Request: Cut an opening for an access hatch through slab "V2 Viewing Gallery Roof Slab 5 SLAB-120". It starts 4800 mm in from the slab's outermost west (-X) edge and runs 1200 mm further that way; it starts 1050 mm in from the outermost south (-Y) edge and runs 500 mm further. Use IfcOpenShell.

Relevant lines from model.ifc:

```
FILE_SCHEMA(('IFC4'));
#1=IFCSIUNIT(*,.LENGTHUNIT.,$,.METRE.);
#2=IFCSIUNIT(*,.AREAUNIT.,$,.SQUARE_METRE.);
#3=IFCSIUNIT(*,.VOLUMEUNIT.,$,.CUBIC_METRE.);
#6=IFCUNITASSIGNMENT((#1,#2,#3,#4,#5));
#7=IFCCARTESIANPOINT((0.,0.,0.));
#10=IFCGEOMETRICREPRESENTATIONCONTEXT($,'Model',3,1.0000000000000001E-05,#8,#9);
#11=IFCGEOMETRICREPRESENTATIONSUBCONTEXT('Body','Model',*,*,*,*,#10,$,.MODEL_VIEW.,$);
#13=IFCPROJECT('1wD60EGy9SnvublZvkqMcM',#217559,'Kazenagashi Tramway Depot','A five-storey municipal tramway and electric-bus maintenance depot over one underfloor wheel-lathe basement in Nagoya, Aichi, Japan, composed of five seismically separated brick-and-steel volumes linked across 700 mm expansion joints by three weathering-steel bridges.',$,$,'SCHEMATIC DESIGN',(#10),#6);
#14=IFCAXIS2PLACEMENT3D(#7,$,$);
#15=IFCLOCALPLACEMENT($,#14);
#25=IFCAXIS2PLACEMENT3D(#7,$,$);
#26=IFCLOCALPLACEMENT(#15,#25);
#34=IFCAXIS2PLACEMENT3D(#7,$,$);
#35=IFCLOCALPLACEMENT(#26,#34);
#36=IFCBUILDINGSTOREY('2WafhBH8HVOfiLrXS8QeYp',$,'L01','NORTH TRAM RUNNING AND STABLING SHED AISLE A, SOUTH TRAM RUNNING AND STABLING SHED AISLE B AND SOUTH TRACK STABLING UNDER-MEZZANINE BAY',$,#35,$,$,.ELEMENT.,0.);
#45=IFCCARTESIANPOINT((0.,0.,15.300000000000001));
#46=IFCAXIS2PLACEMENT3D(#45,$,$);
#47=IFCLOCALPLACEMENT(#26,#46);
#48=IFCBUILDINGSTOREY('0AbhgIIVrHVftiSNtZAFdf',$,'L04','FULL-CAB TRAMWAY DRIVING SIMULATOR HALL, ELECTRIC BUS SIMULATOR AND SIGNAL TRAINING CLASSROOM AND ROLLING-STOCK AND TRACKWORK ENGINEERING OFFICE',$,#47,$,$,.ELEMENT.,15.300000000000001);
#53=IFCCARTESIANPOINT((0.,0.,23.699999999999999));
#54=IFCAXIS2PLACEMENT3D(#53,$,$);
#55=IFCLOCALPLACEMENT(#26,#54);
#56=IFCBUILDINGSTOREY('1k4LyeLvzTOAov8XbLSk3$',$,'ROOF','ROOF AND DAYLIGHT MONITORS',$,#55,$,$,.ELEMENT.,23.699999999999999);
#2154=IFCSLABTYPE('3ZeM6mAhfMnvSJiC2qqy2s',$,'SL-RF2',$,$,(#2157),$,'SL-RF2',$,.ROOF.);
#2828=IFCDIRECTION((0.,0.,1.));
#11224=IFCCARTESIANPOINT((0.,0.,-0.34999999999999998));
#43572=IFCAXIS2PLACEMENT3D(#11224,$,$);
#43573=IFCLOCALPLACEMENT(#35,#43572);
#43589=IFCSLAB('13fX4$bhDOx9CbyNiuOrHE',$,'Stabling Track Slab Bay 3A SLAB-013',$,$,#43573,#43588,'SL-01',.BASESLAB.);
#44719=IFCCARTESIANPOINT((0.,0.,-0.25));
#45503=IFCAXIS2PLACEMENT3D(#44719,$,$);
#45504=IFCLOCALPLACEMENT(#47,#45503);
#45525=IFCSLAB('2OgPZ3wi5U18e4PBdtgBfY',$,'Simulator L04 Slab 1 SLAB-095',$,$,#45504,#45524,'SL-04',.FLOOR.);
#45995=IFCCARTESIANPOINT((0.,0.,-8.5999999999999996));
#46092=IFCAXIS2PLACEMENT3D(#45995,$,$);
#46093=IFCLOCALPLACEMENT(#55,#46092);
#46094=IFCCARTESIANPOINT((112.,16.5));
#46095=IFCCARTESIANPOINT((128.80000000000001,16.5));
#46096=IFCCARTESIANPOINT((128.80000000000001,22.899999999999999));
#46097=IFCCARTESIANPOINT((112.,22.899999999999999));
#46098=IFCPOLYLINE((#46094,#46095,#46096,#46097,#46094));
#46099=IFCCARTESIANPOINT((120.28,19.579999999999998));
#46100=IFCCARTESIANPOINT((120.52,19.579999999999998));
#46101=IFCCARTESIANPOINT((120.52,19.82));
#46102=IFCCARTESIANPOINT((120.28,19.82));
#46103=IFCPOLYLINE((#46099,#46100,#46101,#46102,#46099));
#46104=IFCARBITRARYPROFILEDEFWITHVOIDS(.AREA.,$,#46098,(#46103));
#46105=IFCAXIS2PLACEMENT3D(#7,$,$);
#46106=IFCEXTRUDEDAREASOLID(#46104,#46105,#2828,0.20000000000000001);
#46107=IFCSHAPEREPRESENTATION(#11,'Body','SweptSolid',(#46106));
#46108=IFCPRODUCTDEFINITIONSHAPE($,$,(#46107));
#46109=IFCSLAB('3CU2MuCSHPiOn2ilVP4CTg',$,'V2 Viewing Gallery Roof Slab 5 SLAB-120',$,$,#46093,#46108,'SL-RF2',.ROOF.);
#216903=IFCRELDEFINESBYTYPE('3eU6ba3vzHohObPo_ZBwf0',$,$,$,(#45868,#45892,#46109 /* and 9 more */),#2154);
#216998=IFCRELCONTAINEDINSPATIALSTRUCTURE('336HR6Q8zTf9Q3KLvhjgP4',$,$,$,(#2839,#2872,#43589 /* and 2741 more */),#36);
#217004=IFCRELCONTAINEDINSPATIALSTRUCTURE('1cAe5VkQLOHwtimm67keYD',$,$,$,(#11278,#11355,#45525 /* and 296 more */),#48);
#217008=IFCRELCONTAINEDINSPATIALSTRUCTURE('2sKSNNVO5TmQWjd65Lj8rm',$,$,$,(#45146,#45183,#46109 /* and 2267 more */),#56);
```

```python
import numpy as np
import ifcopenshell
import ifcopenshell.api.feature
import ifcopenshell.api.geometry
import ifcopenshell.api.root
import ifcopenshell.geom
import ifcopenshell.util.placement
import ifcopenshell.util.representation
import ifcopenshell.util.shape
import ifcopenshell.util.unit

model = ifcopenshell.open("model.ifc")
unit_scale = ifcopenshell.util.unit.calculate_unit_scale(model)
settings = ifcopenshell.geom.settings()


def volume(element):
    """Net volume in cubic metres, openings subtracted."""
    shape = ifcopenshell.geom.create_shape(settings, element)
    return ifcopenshell.util.shape.get_volume(shape.geometry)


slab = model.by_id(46109)
before = volume(slab)

# Extent in the slab's own axes, in metres. The edges named are its -X and -Y sides.
slab_shape = ifcopenshell.geom.create_shape(settings, slab)
vertices = ifcopenshell.util.shape.get_vertices(slab_shape.geometry)
x_min, y_min, bottom = vertices.min(axis=0)
top = vertices[:, 2].max()

opening = ifcopenshell.api.root.create_entity(model, ifc_class="IfcOpeningElement", name="Access hatch opening", predefined_type="OPENING")
context = ifcopenshell.util.representation.get_context(model, "Model", "Body", "MODEL_VIEW")
width, depth = 1.2, 0.5
outline = [(0.0, 0.0), (width, 0.0), (width, depth), (0.0, depth), (0.0, 0.0)]
# Overshoot both faces by 50 mm so the cut is clean.
shape = ifcopenshell.api.geometry.add_slab_representation(
    model, context=context, depth=top - bottom + 0.1, polyline=outline
)
ifcopenshell.api.geometry.assign_representation(model, product=opening, representation=shape)

matrix = ifcopenshell.util.placement.get_local_placement(slab.ObjectPlacement)
matrix[:, 3] = matrix @ np.append(np.array([x_min + 4.8, y_min + 1.05, bottom - 0.05]) / unit_scale, 1.0)
ifcopenshell.api.geometry.edit_object_placement(model, product=opening, matrix=matrix, is_si=False)
ifcopenshell.api.feature.add_feature(model, feature=opening, element=slab)

after = volume(slab)

print(f"slab volume {before:.3f} -> {after:.3f} m3")

model.write("model_rev.ifc")
```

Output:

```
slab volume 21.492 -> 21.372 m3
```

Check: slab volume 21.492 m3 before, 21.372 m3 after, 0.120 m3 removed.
